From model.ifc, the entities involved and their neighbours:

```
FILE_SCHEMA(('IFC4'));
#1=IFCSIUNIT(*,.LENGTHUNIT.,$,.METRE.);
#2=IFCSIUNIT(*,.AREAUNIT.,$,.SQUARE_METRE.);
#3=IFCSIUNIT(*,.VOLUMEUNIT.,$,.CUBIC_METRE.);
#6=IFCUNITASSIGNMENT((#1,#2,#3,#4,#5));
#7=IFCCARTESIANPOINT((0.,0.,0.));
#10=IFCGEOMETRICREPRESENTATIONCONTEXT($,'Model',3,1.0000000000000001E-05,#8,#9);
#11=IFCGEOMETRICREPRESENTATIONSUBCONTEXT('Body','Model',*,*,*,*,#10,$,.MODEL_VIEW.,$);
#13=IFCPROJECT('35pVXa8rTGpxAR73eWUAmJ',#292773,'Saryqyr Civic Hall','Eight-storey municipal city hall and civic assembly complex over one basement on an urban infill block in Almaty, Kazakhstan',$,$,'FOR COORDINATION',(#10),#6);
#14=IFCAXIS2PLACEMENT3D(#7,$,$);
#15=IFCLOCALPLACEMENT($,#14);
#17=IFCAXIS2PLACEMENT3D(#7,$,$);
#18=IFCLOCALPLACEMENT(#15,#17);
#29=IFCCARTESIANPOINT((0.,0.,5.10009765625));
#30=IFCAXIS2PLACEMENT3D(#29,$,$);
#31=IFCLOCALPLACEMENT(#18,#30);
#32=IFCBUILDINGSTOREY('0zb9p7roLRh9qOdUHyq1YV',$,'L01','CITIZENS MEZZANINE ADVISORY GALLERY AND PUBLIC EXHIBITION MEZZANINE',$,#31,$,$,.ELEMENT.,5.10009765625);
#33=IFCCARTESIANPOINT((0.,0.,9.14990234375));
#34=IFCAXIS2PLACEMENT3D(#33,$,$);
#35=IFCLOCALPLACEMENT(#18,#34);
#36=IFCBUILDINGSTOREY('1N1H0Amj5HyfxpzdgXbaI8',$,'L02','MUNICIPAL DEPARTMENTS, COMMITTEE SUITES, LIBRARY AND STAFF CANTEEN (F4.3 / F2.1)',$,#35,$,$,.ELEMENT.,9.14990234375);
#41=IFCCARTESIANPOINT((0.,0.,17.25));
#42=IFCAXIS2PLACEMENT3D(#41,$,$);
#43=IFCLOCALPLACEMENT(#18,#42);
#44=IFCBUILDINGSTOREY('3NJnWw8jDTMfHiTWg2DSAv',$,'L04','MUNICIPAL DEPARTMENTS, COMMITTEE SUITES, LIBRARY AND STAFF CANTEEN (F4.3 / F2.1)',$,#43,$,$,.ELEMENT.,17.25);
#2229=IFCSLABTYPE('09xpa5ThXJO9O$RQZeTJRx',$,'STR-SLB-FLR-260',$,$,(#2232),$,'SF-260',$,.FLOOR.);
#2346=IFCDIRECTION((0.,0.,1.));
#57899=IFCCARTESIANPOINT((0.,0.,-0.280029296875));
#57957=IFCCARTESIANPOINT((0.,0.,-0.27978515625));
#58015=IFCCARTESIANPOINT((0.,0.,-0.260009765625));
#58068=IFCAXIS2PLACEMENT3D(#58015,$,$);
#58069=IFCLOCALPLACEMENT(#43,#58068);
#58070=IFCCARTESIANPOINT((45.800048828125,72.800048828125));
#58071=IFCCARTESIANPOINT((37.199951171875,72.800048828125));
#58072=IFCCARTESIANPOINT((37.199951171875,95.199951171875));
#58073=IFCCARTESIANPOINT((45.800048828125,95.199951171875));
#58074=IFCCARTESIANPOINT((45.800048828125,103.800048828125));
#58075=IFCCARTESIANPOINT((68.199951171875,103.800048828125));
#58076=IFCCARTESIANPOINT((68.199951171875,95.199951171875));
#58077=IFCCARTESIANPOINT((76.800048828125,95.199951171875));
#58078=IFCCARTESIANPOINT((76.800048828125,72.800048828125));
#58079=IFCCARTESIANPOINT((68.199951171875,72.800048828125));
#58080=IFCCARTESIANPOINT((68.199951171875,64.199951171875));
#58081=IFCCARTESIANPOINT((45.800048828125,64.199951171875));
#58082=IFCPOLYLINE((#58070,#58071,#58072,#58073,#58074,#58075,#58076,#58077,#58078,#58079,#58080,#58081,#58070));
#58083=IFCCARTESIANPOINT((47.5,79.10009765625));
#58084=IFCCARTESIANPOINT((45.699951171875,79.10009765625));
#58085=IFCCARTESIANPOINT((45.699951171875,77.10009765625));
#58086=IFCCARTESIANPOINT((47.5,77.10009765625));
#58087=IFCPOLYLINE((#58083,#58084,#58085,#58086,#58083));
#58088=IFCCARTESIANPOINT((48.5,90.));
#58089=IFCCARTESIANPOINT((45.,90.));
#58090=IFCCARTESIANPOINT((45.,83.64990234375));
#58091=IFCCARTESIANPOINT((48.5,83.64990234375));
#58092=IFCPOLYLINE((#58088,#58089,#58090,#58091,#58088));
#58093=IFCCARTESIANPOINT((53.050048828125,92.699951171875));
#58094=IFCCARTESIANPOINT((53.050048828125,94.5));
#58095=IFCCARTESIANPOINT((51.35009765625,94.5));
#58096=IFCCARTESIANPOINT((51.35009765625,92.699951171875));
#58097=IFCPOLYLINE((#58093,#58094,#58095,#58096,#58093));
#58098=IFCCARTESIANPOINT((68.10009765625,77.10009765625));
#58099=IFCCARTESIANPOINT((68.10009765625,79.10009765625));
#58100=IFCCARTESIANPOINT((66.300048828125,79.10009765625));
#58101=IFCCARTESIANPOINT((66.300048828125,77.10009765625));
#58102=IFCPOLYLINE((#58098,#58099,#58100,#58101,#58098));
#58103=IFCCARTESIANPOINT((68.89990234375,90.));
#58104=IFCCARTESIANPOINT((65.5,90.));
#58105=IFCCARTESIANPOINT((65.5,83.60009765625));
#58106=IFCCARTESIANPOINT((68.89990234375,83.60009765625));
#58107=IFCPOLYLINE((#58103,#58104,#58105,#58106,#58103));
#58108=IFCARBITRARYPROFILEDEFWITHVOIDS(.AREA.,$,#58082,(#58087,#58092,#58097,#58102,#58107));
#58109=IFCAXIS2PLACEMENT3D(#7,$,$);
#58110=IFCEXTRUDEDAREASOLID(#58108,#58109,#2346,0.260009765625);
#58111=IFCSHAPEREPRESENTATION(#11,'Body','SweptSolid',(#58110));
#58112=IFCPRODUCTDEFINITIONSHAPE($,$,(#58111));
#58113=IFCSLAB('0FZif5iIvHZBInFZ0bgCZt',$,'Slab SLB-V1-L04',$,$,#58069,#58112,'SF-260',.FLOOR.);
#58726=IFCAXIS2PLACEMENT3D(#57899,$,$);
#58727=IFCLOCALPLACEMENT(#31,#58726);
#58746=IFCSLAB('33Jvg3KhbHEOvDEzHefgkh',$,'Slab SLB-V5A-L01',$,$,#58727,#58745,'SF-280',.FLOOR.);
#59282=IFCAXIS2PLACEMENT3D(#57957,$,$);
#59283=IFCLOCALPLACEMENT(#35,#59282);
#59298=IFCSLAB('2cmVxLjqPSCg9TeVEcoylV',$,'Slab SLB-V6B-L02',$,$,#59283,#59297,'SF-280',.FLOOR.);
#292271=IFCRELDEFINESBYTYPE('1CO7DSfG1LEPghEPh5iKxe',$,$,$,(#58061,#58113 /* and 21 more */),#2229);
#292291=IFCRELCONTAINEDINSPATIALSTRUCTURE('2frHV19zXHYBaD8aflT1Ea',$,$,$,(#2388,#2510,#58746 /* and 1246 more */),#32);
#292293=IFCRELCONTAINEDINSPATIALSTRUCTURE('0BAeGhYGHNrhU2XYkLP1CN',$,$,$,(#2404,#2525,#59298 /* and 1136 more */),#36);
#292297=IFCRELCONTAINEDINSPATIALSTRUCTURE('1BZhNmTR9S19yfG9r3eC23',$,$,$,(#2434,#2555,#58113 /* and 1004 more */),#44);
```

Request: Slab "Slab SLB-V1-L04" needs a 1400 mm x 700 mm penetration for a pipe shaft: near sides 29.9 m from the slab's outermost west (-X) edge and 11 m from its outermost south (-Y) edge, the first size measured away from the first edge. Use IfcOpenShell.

```python
import numpy as np
import ifcopenshell
import ifcopenshell.api.feature
import ifcopenshell.api.geometry
import ifcopenshell.api.root
import ifcopenshell.geom
import ifcopenshell.util.placement
import ifcopenshell.util.representation
import ifcopenshell.util.shape
import ifcopenshell.util.unit

model = ifcopenshell.open("model.ifc")
unit_scale = ifcopenshell.util.unit.calculate_unit_scale(model)
settings = ifcopenshell.geom.settings()


def volume(element):
    """Net volume in cubic metres, openings subtracted."""
    shape = ifcopenshell.geom.create_shape(settings, element)
    return ifcopenshell.util.shape.get_volume(shape.geometry)


slab = model.by_guid("0FZif5iIvHZBInFZ0bgCZt")
before = volume(slab)

# Extent in the slab's own axes, in metres. The edges named are its -X and -Y sides.
slab_shape = ifcopenshell.geom.create_shape(settings, slab)
vertices = ifcopenshell.util.shape.get_vertices(slab_shape.geometry)
x_min, y_min, bottom = vertices.min(axis=0)
top = vertices[:, 2].max()

opening = ifcopenshell.api.root.create_entity(model, ifc_class="IfcOpeningElement", name="Pipe shaft opening", predefined_type="OPENING")
context = ifcopenshell.util.representation.get_context(model, "Model", "Body", "MODEL_VIEW")
width, depth = 1.4, 0.7
outline = [(0.0, 0.0), (width, 0.0), (width, depth), (0.0, depth), (0.0, 0.0)]
# Overshoot both faces by 50 mm so the cut is clean.
shape = ifcopenshell.api.geometry.add_slab_representation(
    model, context=context, depth=top - bottom + 0.1, polyline=outline
)
ifcopenshell.api.geometry.assign_representation(model, product=opening, representation=shape)

matrix = ifcopenshell.util.placement.get_local_placement(slab.ObjectPlacement)
matrix[:, 3] = matrix @ np.append(np.array([x_min + 29.9, y_min + 11, bottom - 0.05]) / unit_scale, 1.0)
ifcopenshell.api.geometry.edit_object_placement(model, product=opening, matrix=matrix, is_si=False)
ifcopenshell.api.feature.add_feature(model, feature=opening, element=slab)

after = volume(slab)

print(f"slab volume {before:.3f} -> {after:.3f} m3")

model.write("model_rev.ifc")
```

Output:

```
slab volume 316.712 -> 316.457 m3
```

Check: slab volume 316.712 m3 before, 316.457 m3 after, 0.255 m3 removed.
